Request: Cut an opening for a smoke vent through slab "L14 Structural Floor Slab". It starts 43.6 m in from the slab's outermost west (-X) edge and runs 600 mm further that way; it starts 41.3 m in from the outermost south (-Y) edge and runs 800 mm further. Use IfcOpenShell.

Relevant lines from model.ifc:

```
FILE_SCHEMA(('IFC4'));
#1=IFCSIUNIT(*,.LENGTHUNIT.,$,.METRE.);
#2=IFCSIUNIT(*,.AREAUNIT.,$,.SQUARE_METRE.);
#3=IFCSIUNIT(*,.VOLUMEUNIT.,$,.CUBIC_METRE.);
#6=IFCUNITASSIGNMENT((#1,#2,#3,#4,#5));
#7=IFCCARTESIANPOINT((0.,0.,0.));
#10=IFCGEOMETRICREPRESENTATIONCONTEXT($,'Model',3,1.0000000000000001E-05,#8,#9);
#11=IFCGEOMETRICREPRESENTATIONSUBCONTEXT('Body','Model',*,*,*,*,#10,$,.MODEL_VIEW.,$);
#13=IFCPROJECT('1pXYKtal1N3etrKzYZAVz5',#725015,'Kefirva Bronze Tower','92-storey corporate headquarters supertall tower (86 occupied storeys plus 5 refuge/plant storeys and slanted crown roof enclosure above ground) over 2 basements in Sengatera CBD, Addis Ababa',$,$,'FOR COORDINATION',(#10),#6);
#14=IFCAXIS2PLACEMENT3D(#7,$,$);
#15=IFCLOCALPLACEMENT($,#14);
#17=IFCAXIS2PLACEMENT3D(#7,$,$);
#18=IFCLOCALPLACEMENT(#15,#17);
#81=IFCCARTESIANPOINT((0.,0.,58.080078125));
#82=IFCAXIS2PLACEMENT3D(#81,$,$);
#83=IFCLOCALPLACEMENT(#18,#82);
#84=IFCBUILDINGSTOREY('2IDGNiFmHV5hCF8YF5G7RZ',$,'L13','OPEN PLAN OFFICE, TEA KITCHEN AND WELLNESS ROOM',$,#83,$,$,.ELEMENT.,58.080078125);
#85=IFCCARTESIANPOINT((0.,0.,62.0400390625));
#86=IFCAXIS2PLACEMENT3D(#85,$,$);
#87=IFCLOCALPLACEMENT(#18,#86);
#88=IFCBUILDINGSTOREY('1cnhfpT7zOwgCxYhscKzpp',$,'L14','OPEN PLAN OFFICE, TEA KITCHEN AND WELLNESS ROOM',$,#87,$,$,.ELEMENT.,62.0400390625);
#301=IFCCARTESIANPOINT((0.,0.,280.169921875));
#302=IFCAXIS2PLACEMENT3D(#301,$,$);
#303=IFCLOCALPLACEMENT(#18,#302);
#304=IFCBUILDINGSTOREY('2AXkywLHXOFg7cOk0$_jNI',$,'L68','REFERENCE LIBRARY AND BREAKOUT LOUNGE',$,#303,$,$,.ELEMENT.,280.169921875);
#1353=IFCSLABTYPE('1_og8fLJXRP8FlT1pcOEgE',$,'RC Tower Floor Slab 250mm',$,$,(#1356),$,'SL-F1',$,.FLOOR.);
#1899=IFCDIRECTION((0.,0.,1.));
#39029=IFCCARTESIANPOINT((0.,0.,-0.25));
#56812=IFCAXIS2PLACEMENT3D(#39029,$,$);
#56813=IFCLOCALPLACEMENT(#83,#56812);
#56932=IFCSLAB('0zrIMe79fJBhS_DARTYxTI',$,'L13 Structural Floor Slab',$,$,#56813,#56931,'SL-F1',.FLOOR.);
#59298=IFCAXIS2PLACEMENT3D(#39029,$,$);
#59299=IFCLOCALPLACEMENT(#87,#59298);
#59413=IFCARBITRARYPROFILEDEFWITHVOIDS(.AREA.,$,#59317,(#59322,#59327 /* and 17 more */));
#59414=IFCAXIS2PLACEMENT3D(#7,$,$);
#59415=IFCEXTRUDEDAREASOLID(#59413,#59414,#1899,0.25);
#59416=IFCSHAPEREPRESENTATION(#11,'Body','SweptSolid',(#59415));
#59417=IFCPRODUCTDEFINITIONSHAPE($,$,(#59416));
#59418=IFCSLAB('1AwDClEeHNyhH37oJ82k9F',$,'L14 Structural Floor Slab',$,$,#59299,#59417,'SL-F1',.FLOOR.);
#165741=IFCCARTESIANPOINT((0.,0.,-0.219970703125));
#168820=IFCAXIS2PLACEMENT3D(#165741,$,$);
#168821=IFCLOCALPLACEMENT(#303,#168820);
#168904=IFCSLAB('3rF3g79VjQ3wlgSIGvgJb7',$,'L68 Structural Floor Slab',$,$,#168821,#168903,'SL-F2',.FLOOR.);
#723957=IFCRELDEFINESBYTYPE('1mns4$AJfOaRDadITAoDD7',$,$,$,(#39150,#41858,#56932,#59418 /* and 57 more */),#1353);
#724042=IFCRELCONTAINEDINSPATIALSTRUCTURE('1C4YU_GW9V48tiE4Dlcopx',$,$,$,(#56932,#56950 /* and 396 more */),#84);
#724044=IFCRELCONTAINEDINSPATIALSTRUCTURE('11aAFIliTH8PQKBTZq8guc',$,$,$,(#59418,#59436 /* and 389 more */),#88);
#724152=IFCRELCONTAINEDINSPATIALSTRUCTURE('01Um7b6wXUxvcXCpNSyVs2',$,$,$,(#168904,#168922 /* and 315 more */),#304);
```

```python
import numpy as np
import ifcopenshell
import ifcopenshell.api.feature
import ifcopenshell.api.geometry
import ifcopenshell.api.root
import ifcopenshell.geom
import ifcopenshell.util.placement
import ifcopenshell.util.representation
import ifcopenshell.util.shape
import ifcopenshell.util.unit

model = ifcopenshell.open("model.ifc")
unit_scale = ifcopenshell.util.unit.calculate_unit_scale(model)
settings = ifcopenshell.geom.settings()


def volume(element):
    """Net volume in cubic metres, openings subtracted."""
    shape = ifcopenshell.geom.create_shape(settings, element)
    return ifcopenshell.util.shape.get_volume(shape.geometry)


slab = model.by_guid("1AwDClEeHNyhH37oJ82k9F")
before = volume(slab)

# Extent in the slab's own axes, in metres. The edges named are its -X and -Y sides.
slab_shape = ifcopenshell.geom.create_shape(settings, slab)
vertices = ifcopenshell.util.shape.get_vertices(slab_shape.geometry)
x_min, y_min, bottom = vertices.min(axis=0)
top = vertices[:, 2].max()

opening = ifcopenshell.api.root.create_entity(model, ifc_class="IfcOpeningElement", name="Smoke vent opening", predefined_type="OPENING")
context = ifcopenshell.util.representation.get_context(model, "Model", "Body", "MODEL_VIEW")
width, depth = 0.6, 0.8
outline = [(0.0, 0.0), (width, 0.0), (width, depth), (0.0, depth), (0.0, 0.0)]
# Overshoot both faces by 50 mm so the cut is clean.
shape = ifcopenshell.api.geometry.add_slab_representation(
    model, context=context, depth=top - bottom + 0.1, polyline=outline
)
ifcopenshell.api.geometry.assign_representation(model, product=opening, representation=shape)

matrix = ifcopenshell.util.placement.get_local_placement(slab.ObjectPlacement)
matrix[:, 3] = matrix @ np.append(np.array([x_min + 43.6, y_min + 41.3, bottom - 0.05]) / unit_scale, 1.0)
ifcopenshell.api.geometry.edit_object_placement(model, product=opening, matrix=matrix, is_si=False)
ifcopenshell.api.feature.add_feature(model, feature=opening, element=slab)

after = volume(slab)

print(f"slab volume {before:.3f} -> {after:.3f} m3")

model.write("model_edited.ifc")
```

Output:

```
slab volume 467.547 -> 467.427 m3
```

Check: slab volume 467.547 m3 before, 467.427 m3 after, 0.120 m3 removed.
